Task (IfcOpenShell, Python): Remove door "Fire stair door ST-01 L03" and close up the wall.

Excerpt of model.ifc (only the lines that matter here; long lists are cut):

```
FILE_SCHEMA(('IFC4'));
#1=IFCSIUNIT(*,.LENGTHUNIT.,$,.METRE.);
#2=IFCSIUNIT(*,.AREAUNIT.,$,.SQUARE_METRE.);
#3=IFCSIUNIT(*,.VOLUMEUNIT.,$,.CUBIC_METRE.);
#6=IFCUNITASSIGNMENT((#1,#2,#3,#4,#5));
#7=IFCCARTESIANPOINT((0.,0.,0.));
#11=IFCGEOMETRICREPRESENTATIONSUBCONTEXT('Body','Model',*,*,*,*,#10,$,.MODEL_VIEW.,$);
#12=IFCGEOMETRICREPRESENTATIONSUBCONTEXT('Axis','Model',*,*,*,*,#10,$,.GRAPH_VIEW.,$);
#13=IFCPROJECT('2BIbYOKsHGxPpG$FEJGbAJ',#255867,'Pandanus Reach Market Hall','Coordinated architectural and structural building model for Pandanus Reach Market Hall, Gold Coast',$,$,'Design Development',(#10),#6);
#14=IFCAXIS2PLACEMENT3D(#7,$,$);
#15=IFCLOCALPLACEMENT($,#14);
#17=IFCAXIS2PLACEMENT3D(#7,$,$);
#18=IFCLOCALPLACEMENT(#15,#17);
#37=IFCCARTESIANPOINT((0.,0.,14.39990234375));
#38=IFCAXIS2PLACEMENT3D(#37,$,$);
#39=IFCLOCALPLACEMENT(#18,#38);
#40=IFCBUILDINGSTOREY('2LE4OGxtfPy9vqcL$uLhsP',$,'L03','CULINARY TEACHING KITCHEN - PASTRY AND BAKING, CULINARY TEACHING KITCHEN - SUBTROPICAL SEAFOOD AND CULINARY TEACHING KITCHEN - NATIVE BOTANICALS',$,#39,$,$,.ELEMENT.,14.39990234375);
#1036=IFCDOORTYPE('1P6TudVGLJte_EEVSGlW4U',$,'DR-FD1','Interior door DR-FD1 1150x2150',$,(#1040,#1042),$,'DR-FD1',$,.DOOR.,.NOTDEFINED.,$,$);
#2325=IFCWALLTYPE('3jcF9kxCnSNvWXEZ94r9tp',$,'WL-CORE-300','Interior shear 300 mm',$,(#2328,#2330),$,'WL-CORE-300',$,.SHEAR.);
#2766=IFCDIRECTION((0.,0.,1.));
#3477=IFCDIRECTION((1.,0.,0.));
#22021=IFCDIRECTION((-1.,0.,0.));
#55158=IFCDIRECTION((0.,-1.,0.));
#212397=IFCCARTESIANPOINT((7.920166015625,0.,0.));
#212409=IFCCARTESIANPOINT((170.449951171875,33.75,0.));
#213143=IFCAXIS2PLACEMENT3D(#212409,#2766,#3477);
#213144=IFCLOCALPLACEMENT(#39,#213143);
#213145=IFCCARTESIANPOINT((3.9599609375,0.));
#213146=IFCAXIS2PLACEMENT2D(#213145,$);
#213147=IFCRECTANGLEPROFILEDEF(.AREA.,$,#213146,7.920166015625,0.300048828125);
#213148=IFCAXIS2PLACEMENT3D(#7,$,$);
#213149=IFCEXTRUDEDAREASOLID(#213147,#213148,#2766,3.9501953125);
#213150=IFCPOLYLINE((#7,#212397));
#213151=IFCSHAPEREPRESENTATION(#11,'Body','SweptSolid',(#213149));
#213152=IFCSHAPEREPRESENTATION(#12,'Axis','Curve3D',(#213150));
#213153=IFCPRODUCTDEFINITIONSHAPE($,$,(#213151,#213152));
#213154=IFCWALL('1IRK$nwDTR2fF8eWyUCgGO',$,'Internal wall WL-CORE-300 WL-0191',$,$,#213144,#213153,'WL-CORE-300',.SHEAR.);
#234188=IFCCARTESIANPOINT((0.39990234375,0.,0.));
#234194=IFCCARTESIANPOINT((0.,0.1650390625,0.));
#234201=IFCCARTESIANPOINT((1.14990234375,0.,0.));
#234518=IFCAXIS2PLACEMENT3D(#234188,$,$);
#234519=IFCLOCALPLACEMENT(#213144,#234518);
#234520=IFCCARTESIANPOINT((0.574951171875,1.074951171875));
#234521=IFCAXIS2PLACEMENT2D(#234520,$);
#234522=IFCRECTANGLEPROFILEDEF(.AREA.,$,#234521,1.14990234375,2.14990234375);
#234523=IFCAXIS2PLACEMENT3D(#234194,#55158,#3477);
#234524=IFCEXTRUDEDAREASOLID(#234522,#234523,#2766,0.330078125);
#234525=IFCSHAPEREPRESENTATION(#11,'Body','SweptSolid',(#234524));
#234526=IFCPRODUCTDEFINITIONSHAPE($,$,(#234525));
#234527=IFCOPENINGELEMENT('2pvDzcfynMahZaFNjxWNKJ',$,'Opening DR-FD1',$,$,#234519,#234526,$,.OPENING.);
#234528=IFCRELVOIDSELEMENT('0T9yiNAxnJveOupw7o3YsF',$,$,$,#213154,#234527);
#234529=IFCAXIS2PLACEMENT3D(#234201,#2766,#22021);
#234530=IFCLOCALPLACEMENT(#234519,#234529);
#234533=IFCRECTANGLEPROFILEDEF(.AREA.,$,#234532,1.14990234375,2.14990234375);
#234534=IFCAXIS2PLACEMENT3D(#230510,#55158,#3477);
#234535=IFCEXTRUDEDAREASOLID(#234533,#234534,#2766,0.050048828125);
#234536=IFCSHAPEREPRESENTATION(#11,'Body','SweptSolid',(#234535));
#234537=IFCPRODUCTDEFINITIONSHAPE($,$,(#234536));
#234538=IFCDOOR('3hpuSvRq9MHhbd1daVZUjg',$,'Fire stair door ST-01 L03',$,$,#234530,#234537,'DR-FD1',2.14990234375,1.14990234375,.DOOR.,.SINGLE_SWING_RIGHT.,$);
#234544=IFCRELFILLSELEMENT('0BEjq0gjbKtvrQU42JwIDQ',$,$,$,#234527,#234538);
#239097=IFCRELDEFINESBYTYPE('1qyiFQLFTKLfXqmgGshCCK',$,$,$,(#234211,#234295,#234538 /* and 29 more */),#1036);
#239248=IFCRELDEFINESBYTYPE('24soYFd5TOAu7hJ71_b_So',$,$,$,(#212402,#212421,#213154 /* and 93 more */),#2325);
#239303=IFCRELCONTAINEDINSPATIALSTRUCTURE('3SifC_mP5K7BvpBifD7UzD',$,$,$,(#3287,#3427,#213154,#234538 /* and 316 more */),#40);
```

```python
import ifcopenshell
import ifcopenshell.api.feature
import ifcopenshell.api.root
import ifcopenshell.geom
import ifcopenshell.util.shape

model = ifcopenshell.open("model.ifc")
settings = ifcopenshell.geom.settings()


def volume(element):
    """Net volume in cubic metres, openings subtracted."""
    shape = ifcopenshell.geom.create_shape(settings, element)
    return ifcopenshell.util.shape.get_volume(shape.geometry)


door = model.by_guid("3hpuSvRq9MHhbd1daVZUjg")
opening = door.FillsVoids[0].RelatingOpeningElement
wall = opening.VoidsElements[0].RelatingBuildingElement
before = volume(wall)

ifcopenshell.api.root.remove_product(model, product=door)
ifcopenshell.api.feature.remove_feature(model, feature=opening)

after = volume(wall)

print(f"wall volume {before:.3f} -> {after:.3f} m3")

model.write("model_rev.ifc")
```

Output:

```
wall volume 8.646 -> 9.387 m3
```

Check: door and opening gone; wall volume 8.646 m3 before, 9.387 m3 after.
